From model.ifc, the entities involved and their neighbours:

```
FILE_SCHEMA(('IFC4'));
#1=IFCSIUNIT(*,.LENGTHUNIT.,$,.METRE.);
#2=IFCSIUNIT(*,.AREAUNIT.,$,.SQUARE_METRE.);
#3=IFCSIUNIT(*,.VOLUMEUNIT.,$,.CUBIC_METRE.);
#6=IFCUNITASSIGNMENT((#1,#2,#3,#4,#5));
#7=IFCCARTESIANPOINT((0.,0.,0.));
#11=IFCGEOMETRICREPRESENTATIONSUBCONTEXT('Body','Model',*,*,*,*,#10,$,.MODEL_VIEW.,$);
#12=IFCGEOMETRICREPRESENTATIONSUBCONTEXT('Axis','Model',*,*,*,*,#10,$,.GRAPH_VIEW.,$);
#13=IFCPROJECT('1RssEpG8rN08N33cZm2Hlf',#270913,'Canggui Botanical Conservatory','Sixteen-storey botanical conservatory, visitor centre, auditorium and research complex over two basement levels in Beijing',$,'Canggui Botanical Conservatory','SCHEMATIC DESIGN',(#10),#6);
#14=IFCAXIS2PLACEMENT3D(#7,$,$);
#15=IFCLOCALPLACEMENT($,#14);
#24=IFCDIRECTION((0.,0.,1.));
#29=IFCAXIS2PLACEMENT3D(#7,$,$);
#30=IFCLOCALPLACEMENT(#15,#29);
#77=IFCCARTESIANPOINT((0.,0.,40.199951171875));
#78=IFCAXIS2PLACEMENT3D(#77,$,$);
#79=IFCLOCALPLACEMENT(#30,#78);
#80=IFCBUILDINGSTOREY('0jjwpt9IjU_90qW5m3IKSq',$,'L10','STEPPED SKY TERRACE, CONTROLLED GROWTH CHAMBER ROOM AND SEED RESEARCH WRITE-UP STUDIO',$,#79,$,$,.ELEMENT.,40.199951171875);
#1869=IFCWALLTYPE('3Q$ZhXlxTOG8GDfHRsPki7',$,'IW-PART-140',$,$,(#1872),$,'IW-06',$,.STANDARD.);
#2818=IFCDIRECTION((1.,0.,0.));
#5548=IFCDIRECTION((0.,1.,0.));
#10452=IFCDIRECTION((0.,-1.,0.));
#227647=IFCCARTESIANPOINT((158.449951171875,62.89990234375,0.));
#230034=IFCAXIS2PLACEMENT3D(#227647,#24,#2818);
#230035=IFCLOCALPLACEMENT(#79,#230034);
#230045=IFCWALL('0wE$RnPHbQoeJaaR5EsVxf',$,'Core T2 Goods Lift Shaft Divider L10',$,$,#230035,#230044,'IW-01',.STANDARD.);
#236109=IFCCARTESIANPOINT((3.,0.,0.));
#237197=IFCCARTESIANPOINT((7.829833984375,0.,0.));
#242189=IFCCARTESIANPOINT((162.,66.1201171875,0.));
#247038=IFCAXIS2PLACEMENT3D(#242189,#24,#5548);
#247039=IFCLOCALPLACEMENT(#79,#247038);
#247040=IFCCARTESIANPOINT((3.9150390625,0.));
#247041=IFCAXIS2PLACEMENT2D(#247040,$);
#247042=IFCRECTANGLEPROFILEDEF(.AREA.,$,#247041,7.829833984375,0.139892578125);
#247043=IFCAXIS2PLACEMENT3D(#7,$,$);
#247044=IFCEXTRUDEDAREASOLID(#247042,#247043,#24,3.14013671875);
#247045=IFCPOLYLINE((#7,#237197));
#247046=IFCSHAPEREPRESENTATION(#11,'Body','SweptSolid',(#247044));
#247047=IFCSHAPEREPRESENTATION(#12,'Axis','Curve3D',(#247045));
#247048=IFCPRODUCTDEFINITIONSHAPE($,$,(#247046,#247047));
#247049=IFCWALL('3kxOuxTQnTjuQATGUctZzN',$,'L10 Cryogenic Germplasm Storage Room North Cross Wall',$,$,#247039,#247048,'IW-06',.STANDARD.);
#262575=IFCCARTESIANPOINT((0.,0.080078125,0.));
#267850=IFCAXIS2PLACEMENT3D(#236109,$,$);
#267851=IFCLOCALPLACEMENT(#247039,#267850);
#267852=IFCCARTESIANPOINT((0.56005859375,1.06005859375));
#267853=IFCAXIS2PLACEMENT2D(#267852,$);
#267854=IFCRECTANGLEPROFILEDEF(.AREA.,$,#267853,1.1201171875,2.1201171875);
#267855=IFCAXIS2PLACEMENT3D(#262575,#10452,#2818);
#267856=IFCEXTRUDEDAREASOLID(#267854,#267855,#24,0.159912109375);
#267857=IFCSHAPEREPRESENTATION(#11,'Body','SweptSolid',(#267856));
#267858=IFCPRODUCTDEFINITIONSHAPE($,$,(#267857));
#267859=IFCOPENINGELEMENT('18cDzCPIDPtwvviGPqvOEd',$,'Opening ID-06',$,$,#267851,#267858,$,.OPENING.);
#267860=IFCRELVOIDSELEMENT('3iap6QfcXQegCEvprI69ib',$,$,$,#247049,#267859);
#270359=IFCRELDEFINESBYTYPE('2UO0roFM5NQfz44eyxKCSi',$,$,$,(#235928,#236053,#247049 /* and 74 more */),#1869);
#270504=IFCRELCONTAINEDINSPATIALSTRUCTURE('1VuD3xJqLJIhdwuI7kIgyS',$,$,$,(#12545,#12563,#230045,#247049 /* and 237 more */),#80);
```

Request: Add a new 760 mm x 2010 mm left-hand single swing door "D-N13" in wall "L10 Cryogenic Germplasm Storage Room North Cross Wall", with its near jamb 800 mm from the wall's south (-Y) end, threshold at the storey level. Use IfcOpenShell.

```python
import numpy as np
import ifcopenshell
import ifcopenshell.api.feature
import ifcopenshell.api.geometry
import ifcopenshell.api.root
import ifcopenshell.api.spatial
import ifcopenshell.geom
import ifcopenshell.util.element
import ifcopenshell.util.placement
import ifcopenshell.util.representation
import ifcopenshell.util.shape
import ifcopenshell.util.unit

model = ifcopenshell.open("model.ifc")
unit_scale = ifcopenshell.util.unit.calculate_unit_scale(model)
settings = ifcopenshell.geom.settings()


def volume(element):
    """Net volume in cubic metres, openings subtracted."""
    shape = ifcopenshell.geom.create_shape(settings, element)
    return ifcopenshell.util.shape.get_volume(shape.geometry)


wall = model.by_guid("3kxOuxTQnTjuQATGUctZzN")
storey = ifcopenshell.util.element.get_container(wall, ifc_class="IfcBuildingStorey")
context = ifcopenshell.util.representation.get_context(model, "Model", "Body", "MODEL_VIEW")
before = volume(wall)

width, height, from_end, sill = 0.76, 2.01, 0.8, 0.0  # metres

# The wall runs along its own X axis, and the end named is its -X end.
wall_shape = ifcopenshell.geom.create_shape(settings, wall)
x, y, z = ifcopenshell.util.shape.get_vertices(wall_shape.geometry).T
start = x.min() + from_end
face, thickness = float(y.min()), float(y.max() - y.min())
wall_matrix = ifcopenshell.util.placement.get_local_placement(wall.ObjectPlacement)
level = ifcopenshell.util.placement.get_local_placement(storey.ObjectPlacement)[2, 3]


def in_wall(x, y):
    """Placement at x, y metres in the wall's axes, at sill height."""
    matrix = wall_matrix.copy()
    matrix[:, 3] = wall_matrix @ np.array([x / unit_scale, y / unit_scale, 0.0, 1.0])
    matrix[2, 3] = level + sill / unit_scale
    return matrix


# Opening: a box that overshoots both wall faces by 50 mm.
opening = ifcopenshell.api.root.create_entity(model, ifc_class="IfcOpeningElement", predefined_type="OPENING")
box = ifcopenshell.api.geometry.add_wall_representation(
    model, context=context, length=width, height=height, thickness=thickness + 0.1
)
ifcopenshell.api.geometry.assign_representation(model, product=opening, representation=box)
ifcopenshell.api.geometry.edit_object_placement(model, product=opening, matrix=in_wall(start, face - 0.05), is_si=False)
ifcopenshell.api.feature.add_feature(model, feature=opening, element=wall)

door = ifcopenshell.api.root.create_entity(model, ifc_class="IfcDoor", name="D-N13", predefined_type="DOOR")
door.OverallWidth, door.OverallHeight = width / unit_scale, height / unit_scale
door.OperationType = "SINGLE_SWING_LEFT"
body = ifcopenshell.api.geometry.add_door_representation(
    model,
    context=context,
    overall_width=door.OverallWidth,
    overall_height=door.OverallHeight,
    operation_type="SINGLE_SWING_LEFT",
    lining_properties={"LiningDepth": thickness / unit_scale, "ThresholdDepth": thickness / unit_scale},
)
ifcopenshell.api.geometry.assign_representation(model, product=door, representation=body)
ifcopenshell.api.spatial.assign_container(model, products=[door], relating_structure=storey)
ifcopenshell.api.feature.add_filling(model, opening=opening, element=door)

# The lining spans the wall, so the door starts at the wall face.
ifcopenshell.api.geometry.edit_object_placement(model, product=door, matrix=in_wall(start, face), is_si=False)

after = volume(wall)

print(f"wall volume {before:.3f} -> {after:.3f} m3")

model.write("model_rev.ifc")
```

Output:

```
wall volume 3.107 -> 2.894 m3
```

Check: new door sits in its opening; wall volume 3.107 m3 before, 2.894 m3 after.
